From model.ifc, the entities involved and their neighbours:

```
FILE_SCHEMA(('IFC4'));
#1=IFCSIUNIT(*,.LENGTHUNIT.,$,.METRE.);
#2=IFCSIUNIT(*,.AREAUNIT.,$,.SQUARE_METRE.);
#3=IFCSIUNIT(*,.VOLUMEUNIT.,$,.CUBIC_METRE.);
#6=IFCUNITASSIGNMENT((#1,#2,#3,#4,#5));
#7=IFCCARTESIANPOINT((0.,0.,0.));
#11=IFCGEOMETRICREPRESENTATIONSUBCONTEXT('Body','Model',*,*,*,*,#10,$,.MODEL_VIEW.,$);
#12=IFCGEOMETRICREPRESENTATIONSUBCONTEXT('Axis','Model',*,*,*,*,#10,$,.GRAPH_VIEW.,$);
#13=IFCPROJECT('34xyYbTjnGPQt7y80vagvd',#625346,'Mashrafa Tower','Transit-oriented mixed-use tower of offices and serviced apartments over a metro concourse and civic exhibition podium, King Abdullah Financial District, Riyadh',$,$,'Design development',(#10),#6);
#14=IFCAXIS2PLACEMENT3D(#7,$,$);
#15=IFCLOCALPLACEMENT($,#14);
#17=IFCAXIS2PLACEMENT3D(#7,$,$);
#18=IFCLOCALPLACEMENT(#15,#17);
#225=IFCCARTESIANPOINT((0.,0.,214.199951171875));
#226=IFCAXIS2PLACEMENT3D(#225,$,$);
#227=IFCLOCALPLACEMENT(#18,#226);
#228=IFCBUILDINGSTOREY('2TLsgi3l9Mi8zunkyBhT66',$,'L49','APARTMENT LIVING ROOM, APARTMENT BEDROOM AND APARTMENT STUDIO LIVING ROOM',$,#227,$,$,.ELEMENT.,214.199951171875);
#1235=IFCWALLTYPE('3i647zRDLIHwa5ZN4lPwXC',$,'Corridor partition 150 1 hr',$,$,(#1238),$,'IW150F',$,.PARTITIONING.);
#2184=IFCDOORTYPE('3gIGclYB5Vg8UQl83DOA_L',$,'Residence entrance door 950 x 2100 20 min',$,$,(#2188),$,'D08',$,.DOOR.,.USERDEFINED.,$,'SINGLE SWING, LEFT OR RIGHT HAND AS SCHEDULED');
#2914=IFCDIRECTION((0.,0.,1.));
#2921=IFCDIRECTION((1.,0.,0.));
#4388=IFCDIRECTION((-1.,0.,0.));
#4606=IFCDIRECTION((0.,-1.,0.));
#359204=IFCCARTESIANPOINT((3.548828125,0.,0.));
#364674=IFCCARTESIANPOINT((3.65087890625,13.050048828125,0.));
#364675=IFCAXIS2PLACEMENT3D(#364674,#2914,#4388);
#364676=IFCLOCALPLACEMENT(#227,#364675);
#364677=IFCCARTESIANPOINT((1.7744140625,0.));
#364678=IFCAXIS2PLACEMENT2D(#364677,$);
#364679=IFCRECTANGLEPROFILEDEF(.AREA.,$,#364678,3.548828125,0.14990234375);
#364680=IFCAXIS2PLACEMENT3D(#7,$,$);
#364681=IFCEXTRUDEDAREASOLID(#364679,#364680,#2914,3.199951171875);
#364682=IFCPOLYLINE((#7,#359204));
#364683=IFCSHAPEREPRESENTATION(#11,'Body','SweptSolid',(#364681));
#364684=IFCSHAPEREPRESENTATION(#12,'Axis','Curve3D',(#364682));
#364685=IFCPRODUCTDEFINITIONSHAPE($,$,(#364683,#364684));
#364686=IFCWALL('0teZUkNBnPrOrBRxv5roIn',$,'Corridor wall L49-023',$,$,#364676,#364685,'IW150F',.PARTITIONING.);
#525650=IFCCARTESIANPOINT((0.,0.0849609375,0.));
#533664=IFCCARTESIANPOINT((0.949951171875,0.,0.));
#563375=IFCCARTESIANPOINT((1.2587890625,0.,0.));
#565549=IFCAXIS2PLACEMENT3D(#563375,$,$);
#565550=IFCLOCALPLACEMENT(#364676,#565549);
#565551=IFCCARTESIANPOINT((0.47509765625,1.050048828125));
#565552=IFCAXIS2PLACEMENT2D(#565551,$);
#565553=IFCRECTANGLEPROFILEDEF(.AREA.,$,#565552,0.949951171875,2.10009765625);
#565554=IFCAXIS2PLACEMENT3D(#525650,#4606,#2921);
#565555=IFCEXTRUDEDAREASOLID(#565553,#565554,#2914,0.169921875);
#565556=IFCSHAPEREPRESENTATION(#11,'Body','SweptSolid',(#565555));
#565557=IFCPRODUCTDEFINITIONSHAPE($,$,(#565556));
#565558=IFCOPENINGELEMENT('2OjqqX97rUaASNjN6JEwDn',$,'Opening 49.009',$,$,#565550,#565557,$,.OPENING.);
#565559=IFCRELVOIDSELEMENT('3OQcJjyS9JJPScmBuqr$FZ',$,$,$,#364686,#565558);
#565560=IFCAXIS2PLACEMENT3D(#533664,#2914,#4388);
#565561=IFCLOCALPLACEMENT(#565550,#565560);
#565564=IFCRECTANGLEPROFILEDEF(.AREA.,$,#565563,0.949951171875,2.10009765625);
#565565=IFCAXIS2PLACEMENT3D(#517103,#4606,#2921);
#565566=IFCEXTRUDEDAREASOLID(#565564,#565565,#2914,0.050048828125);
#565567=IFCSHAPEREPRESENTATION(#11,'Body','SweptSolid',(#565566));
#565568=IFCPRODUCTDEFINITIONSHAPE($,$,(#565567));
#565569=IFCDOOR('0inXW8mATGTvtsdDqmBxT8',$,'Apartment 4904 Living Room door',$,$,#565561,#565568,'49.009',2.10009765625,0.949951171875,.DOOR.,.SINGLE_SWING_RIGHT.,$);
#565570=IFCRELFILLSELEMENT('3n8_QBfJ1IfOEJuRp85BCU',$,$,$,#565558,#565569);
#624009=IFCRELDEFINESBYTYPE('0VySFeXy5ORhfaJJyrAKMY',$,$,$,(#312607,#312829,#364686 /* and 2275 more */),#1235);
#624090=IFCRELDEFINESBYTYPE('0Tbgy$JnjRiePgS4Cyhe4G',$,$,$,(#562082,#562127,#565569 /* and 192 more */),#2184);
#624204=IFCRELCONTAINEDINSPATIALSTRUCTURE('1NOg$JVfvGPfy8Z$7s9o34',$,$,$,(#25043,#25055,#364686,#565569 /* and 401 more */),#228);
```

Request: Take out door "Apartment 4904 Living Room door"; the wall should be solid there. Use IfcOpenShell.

```python
import ifcopenshell
import ifcopenshell.api.feature
import ifcopenshell.api.root
import ifcopenshell.geom
import ifcopenshell.util.shape

model = ifcopenshell.open("model.ifc")
settings = ifcopenshell.geom.settings()


def volume(element):
    """Net volume in cubic metres, openings subtracted."""
    shape = ifcopenshell.geom.create_shape(settings, element)
    return ifcopenshell.util.shape.get_volume(shape.geometry)


door = model.by_id(565569)
opening = door.FillsVoids[0].RelatingOpeningElement
wall = opening.VoidsElements[0].RelatingBuildingElement
before = volume(wall)

ifcopenshell.api.root.remove_product(model, product=door)
ifcopenshell.api.feature.remove_feature(model, feature=opening)

after = volume(wall)

print(f"wall volume {before:.3f} -> {after:.3f} m3")

model.write("model_v2.ifc")
```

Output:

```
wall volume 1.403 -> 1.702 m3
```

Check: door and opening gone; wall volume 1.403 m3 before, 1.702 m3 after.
